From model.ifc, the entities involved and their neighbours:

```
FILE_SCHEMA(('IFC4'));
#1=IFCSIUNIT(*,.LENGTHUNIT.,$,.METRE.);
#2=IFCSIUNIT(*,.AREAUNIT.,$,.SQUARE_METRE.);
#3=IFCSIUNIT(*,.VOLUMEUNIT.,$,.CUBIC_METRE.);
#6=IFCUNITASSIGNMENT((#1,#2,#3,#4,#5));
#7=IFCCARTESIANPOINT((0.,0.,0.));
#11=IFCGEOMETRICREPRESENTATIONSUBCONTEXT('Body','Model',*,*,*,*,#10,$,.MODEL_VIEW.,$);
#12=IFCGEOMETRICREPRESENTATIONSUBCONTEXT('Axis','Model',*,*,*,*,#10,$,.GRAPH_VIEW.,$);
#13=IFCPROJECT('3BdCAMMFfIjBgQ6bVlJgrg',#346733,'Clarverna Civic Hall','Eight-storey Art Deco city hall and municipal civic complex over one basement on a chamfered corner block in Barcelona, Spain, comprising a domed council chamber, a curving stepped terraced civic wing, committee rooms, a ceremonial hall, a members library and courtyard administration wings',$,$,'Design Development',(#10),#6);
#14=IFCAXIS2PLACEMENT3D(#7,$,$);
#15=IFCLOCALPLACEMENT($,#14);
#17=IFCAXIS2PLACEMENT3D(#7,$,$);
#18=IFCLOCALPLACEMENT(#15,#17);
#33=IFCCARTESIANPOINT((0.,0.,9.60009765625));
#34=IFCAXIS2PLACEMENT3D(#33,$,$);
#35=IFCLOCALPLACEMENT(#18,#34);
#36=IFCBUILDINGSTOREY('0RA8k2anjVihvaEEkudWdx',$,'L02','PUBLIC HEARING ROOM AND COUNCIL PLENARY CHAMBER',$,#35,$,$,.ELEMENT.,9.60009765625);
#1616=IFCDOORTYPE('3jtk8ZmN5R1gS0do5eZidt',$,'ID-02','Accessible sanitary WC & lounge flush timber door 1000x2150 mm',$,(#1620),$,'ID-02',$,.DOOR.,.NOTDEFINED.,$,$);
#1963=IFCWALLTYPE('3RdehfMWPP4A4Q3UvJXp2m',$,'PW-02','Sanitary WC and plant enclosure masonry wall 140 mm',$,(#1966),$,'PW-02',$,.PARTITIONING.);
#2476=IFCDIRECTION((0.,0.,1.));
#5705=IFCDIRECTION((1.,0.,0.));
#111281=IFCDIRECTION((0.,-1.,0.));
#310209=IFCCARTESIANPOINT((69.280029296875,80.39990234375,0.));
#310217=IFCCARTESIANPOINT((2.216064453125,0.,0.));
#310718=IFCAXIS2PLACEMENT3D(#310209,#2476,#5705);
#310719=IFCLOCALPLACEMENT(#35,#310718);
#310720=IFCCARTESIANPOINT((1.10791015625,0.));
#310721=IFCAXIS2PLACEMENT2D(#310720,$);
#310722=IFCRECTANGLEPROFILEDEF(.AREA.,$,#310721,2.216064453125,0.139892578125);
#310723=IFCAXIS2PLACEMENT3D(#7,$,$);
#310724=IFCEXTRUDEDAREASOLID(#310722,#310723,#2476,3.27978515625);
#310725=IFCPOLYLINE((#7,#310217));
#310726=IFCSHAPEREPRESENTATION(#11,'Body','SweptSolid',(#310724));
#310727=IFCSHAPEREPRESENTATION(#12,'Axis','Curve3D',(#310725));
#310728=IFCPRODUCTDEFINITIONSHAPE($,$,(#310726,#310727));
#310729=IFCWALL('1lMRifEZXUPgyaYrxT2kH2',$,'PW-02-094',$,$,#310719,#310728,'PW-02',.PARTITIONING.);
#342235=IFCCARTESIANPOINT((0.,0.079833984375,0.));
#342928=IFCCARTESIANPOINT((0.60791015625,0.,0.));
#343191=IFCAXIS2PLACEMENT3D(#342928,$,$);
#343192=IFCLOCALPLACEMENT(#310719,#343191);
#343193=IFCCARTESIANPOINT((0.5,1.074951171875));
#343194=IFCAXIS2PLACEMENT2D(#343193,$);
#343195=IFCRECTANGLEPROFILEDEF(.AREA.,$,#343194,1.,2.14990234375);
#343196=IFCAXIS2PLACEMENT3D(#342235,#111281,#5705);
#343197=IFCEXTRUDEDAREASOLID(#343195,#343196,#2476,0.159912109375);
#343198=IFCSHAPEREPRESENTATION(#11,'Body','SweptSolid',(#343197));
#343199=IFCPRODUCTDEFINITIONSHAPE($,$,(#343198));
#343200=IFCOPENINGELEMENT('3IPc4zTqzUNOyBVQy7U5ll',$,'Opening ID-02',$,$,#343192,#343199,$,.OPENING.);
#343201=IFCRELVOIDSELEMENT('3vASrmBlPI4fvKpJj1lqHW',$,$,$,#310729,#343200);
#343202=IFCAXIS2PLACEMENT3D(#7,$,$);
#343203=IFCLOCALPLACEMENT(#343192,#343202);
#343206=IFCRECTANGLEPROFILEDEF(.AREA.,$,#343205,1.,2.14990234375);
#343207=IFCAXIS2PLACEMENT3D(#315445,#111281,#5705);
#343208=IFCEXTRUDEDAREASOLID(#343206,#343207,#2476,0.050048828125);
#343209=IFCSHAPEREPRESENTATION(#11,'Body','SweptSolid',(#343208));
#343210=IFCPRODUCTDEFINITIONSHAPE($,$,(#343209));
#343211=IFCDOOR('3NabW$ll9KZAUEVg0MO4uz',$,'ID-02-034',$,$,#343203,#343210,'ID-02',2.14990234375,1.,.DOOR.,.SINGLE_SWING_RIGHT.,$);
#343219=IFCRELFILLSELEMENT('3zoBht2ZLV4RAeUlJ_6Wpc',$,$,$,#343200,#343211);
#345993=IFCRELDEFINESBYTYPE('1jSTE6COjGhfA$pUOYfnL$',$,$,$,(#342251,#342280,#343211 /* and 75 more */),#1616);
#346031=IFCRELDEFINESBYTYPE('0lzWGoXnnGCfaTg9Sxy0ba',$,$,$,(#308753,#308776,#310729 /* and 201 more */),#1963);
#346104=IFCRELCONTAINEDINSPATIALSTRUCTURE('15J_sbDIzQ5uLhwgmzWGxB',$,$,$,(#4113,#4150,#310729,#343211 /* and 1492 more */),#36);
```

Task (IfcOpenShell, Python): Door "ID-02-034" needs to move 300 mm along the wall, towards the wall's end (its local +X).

```python
import ifcopenshell
import ifcopenshell.api.geometry
import ifcopenshell.util.placement

model = ifcopenshell.open("model.ifc")

door = model.by_guid("3NabW$ll9KZAUEVg0MO4uz")
opening = door.FillsVoids[0].RelatingOpeningElement
wall = opening.VoidsElements[0].RelatingBuildingElement

wall_matrix = ifcopenshell.util.placement.get_local_placement(wall.ObjectPlacement)
shift = wall_matrix[:3, 0] * 0.3
before = ifcopenshell.util.placement.get_local_placement(door.ObjectPlacement)[:3, 3].copy()

# The door is placed relative to its opening, so it follows when the opening moves.
matrix = ifcopenshell.util.placement.get_local_placement(opening.ObjectPlacement)
matrix[:3, 3] += shift
ifcopenshell.api.geometry.edit_object_placement(
    model, product=opening, matrix=matrix, is_si=False, should_transform_children=True
)

after = ifcopenshell.util.placement.get_local_placement(door.ObjectPlacement)[:3, 3]
print("door moved by", (after - before).round(3) + 0.0)

model.write("model_updated.ifc")
```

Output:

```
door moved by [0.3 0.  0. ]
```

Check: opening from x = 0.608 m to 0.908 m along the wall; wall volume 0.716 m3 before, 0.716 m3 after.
